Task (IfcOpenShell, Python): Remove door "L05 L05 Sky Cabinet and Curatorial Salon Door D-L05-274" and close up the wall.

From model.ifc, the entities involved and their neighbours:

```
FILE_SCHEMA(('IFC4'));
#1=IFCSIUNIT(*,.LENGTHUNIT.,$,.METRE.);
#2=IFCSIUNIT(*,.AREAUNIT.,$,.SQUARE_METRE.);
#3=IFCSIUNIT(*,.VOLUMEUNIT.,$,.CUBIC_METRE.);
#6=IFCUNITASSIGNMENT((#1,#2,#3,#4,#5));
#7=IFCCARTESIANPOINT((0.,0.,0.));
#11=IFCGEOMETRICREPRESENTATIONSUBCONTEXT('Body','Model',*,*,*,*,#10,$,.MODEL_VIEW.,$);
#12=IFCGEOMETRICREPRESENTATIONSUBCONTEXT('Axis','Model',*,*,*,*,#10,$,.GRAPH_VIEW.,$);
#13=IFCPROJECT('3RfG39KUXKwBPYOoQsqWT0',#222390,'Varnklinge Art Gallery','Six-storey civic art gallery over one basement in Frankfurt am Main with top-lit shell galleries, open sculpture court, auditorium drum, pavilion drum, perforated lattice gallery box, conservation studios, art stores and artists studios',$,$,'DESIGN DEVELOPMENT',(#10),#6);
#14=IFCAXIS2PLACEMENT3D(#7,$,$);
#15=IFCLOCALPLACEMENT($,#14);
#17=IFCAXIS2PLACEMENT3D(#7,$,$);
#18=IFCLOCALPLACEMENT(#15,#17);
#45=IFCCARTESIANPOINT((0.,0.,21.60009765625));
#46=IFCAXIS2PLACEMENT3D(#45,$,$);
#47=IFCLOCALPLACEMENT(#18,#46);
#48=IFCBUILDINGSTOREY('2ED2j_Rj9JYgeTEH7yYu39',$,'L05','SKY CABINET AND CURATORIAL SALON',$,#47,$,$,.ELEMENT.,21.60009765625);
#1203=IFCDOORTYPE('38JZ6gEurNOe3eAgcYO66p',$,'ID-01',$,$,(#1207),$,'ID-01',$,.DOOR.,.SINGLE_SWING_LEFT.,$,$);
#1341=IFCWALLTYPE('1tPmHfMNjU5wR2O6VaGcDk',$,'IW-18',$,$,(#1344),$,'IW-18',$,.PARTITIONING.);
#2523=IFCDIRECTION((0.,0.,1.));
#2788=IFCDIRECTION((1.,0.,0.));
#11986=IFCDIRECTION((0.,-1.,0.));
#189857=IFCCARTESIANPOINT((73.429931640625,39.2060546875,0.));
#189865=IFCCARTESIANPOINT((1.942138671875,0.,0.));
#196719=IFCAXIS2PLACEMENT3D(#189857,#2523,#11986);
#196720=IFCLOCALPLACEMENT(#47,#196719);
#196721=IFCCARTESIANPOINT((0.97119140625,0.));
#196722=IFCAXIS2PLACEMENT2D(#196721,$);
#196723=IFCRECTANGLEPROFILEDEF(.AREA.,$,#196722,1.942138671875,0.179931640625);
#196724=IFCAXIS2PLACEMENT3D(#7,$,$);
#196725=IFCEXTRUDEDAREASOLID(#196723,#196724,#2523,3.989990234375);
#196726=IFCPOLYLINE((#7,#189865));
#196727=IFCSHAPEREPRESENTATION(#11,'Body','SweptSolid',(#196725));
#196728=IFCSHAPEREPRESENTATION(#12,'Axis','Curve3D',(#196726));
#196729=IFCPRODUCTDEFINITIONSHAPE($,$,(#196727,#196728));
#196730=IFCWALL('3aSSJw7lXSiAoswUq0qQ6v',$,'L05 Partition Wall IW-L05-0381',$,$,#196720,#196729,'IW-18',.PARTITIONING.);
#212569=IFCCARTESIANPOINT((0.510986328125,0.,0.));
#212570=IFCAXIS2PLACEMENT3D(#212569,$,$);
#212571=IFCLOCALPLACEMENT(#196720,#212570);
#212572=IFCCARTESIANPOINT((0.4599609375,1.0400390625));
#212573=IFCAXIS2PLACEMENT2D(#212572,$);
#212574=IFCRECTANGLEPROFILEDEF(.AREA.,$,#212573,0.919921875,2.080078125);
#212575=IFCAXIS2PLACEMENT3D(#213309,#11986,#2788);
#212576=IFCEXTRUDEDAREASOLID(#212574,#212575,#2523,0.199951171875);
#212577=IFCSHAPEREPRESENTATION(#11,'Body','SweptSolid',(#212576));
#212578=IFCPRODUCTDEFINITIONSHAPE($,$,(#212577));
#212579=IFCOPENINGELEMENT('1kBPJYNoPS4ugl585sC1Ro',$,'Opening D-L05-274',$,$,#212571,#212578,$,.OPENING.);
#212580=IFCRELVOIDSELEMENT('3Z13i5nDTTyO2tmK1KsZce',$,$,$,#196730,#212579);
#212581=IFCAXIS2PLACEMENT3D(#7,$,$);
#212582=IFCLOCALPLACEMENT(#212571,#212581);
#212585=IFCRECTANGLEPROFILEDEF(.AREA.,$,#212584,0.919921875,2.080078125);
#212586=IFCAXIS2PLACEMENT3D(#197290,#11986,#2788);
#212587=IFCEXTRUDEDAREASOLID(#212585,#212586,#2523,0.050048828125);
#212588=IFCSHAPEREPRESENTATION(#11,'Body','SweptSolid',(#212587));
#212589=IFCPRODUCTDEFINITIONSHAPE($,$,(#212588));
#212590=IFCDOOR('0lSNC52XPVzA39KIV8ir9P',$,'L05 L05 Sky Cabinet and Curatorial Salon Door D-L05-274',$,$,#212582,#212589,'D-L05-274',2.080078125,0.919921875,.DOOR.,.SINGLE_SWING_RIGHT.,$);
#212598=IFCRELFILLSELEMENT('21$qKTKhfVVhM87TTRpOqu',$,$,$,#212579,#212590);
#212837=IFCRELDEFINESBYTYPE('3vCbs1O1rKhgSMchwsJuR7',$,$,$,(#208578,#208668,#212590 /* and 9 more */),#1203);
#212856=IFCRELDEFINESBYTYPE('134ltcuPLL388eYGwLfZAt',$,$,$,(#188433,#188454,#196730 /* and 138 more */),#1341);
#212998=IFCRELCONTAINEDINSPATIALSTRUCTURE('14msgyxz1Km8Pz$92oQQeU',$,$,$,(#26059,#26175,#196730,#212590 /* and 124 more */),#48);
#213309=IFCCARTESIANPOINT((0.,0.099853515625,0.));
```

```python
import ifcopenshell
import ifcopenshell.api.feature
import ifcopenshell.api.root
import ifcopenshell.geom
import ifcopenshell.util.shape

model = ifcopenshell.open("model.ifc")
settings = ifcopenshell.geom.settings()


def volume(element):
    """Net volume in cubic metres, openings subtracted."""
    shape = ifcopenshell.geom.create_shape(settings, element)
    return ifcopenshell.util.shape.get_volume(shape.geometry)


door = model.by_guid("0lSNC52XPVzA39KIV8ir9P")
opening = door.FillsVoids[0].RelatingOpeningElement
wall = opening.VoidsElements[0].RelatingBuildingElement
before = volume(wall)

ifcopenshell.api.root.remove_product(model, product=door)
ifcopenshell.api.feature.remove_feature(model, feature=opening)

after = volume(wall)

print(f"wall volume {before:.3f} -> {after:.3f} m3")

model.write("model_rev.ifc")
```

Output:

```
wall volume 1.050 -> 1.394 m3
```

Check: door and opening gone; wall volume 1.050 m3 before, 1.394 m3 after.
